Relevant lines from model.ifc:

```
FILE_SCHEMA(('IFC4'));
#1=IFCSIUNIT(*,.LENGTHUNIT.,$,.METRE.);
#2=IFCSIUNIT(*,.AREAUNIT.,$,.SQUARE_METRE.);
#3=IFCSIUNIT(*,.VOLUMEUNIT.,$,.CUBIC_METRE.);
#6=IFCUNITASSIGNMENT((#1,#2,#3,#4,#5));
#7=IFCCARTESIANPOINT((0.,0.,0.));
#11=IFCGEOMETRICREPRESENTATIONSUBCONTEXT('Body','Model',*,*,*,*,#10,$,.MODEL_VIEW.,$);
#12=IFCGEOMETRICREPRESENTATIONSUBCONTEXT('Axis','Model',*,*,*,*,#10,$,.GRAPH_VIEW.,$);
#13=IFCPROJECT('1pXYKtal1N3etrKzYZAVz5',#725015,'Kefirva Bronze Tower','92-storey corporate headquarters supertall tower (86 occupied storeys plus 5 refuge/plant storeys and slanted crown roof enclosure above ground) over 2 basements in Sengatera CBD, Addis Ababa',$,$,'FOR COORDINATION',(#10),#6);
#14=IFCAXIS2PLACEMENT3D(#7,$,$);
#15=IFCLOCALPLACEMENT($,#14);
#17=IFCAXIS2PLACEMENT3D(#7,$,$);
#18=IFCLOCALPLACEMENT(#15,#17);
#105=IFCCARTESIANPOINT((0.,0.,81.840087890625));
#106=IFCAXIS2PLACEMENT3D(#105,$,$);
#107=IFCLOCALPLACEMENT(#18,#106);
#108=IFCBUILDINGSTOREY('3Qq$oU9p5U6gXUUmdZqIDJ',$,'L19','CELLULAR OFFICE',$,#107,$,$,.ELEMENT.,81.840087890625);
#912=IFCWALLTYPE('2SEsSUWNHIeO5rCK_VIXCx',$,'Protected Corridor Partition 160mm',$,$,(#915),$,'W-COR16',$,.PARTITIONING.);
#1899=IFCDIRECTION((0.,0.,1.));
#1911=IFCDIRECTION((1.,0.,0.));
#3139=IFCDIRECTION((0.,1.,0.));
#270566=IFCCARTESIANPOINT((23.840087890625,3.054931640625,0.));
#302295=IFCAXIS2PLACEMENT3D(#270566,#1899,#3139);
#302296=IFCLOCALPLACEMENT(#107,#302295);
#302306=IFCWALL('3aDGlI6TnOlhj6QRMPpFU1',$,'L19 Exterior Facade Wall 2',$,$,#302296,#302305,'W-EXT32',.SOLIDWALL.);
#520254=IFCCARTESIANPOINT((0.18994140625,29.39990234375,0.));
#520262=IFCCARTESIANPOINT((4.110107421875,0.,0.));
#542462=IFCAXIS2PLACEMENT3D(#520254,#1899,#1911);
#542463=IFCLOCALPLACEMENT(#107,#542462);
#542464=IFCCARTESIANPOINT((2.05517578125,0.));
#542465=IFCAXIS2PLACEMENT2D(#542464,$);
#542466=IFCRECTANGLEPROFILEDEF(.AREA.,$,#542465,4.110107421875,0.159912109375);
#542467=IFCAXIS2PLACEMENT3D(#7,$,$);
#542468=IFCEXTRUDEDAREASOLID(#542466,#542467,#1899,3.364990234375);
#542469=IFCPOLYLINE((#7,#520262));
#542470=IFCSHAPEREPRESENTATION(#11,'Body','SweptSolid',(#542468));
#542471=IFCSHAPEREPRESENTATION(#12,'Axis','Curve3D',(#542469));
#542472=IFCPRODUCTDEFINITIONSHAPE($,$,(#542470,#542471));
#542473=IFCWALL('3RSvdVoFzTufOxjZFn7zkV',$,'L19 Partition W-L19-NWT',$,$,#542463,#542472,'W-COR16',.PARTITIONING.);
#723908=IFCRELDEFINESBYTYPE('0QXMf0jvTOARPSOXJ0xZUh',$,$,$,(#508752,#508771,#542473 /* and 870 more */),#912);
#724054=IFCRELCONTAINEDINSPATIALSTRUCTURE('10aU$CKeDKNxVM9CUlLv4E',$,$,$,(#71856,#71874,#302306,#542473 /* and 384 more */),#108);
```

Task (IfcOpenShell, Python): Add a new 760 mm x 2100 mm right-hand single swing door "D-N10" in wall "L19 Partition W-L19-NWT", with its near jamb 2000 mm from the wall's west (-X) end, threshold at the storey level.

```python
import numpy as np
import ifcopenshell
import ifcopenshell.api.feature
import ifcopenshell.api.geometry
import ifcopenshell.api.root
import ifcopenshell.api.spatial
import ifcopenshell.geom
import ifcopenshell.util.element
import ifcopenshell.util.placement
import ifcopenshell.util.representation
import ifcopenshell.util.shape
import ifcopenshell.util.unit

model = ifcopenshell.open("model.ifc")
unit_scale = ifcopenshell.util.unit.calculate_unit_scale(model)
settings = ifcopenshell.geom.settings()


def volume(element):
    """Net volume in cubic metres, openings subtracted."""
    shape = ifcopenshell.geom.create_shape(settings, element)
    return ifcopenshell.util.shape.get_volume(shape.geometry)


wall = model.by_guid("3RSvdVoFzTufOxjZFn7zkV")
storey = ifcopenshell.util.element.get_container(wall, ifc_class="IfcBuildingStorey")
context = ifcopenshell.util.representation.get_context(model, "Model", "Body", "MODEL_VIEW")
before = volume(wall)

width, height, from_end, sill = 0.76, 2.1, 2, 0.0  # metres

# The wall runs along its own X axis, and the end named is its -X end.
wall_shape = ifcopenshell.geom.create_shape(settings, wall)
x, y, z = ifcopenshell.util.shape.get_vertices(wall_shape.geometry).T
start = x.min() + from_end
face, thickness = float(y.min()), float(y.max() - y.min())
wall_matrix = ifcopenshell.util.placement.get_local_placement(wall.ObjectPlacement)
level = ifcopenshell.util.placement.get_local_placement(storey.ObjectPlacement)[2, 3]


def in_wall(x, y):
    """Placement at x, y metres in the wall's axes, at sill height."""
    matrix = wall_matrix.copy()
    matrix[:, 3] = wall_matrix @ np.array([x / unit_scale, y / unit_scale, 0.0, 1.0])
    matrix[2, 3] = level + sill / unit_scale
    return matrix


# Opening: a box that overshoots both wall faces by 50 mm.
opening = ifcopenshell.api.root.create_entity(model, ifc_class="IfcOpeningElement", predefined_type="OPENING")
box = ifcopenshell.api.geometry.add_wall_representation(
    model, context=context, length=width, height=height, thickness=thickness + 0.1
)
ifcopenshell.api.geometry.assign_representation(model, product=opening, representation=box)
ifcopenshell.api.geometry.edit_object_placement(model, product=opening, matrix=in_wall(start, face - 0.05), is_si=False)
ifcopenshell.api.feature.add_feature(model, feature=opening, element=wall)

door = ifcopenshell.api.root.create_entity(model, ifc_class="IfcDoor", name="D-N10", predefined_type="DOOR")
door.OverallWidth, door.OverallHeight = width / unit_scale, height / unit_scale
door.OperationType = "SINGLE_SWING_RIGHT"
body = ifcopenshell.api.geometry.add_door_representation(
    model,
    context=context,
    overall_width=door.OverallWidth,
    overall_height=door.OverallHeight,
    operation_type="SINGLE_SWING_RIGHT",
    lining_properties={"LiningDepth": thickness / unit_scale, "ThresholdDepth": thickness / unit_scale},
)
ifcopenshell.api.geometry.assign_representation(model, product=door, representation=body)
ifcopenshell.api.spatial.assign_container(model, products=[door], relating_structure=storey)
ifcopenshell.api.feature.add_filling(model, opening=opening, element=door)

# The lining spans the wall, so the door starts at the wall face.
ifcopenshell.api.geometry.edit_object_placement(model, product=door, matrix=in_wall(start, face), is_si=False)

after = volume(wall)

print(f"wall volume {before:.3f} -> {after:.3f} m3")

model.write("model_edited.ifc")
```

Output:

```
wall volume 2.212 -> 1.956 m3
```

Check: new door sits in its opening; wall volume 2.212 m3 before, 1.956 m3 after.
